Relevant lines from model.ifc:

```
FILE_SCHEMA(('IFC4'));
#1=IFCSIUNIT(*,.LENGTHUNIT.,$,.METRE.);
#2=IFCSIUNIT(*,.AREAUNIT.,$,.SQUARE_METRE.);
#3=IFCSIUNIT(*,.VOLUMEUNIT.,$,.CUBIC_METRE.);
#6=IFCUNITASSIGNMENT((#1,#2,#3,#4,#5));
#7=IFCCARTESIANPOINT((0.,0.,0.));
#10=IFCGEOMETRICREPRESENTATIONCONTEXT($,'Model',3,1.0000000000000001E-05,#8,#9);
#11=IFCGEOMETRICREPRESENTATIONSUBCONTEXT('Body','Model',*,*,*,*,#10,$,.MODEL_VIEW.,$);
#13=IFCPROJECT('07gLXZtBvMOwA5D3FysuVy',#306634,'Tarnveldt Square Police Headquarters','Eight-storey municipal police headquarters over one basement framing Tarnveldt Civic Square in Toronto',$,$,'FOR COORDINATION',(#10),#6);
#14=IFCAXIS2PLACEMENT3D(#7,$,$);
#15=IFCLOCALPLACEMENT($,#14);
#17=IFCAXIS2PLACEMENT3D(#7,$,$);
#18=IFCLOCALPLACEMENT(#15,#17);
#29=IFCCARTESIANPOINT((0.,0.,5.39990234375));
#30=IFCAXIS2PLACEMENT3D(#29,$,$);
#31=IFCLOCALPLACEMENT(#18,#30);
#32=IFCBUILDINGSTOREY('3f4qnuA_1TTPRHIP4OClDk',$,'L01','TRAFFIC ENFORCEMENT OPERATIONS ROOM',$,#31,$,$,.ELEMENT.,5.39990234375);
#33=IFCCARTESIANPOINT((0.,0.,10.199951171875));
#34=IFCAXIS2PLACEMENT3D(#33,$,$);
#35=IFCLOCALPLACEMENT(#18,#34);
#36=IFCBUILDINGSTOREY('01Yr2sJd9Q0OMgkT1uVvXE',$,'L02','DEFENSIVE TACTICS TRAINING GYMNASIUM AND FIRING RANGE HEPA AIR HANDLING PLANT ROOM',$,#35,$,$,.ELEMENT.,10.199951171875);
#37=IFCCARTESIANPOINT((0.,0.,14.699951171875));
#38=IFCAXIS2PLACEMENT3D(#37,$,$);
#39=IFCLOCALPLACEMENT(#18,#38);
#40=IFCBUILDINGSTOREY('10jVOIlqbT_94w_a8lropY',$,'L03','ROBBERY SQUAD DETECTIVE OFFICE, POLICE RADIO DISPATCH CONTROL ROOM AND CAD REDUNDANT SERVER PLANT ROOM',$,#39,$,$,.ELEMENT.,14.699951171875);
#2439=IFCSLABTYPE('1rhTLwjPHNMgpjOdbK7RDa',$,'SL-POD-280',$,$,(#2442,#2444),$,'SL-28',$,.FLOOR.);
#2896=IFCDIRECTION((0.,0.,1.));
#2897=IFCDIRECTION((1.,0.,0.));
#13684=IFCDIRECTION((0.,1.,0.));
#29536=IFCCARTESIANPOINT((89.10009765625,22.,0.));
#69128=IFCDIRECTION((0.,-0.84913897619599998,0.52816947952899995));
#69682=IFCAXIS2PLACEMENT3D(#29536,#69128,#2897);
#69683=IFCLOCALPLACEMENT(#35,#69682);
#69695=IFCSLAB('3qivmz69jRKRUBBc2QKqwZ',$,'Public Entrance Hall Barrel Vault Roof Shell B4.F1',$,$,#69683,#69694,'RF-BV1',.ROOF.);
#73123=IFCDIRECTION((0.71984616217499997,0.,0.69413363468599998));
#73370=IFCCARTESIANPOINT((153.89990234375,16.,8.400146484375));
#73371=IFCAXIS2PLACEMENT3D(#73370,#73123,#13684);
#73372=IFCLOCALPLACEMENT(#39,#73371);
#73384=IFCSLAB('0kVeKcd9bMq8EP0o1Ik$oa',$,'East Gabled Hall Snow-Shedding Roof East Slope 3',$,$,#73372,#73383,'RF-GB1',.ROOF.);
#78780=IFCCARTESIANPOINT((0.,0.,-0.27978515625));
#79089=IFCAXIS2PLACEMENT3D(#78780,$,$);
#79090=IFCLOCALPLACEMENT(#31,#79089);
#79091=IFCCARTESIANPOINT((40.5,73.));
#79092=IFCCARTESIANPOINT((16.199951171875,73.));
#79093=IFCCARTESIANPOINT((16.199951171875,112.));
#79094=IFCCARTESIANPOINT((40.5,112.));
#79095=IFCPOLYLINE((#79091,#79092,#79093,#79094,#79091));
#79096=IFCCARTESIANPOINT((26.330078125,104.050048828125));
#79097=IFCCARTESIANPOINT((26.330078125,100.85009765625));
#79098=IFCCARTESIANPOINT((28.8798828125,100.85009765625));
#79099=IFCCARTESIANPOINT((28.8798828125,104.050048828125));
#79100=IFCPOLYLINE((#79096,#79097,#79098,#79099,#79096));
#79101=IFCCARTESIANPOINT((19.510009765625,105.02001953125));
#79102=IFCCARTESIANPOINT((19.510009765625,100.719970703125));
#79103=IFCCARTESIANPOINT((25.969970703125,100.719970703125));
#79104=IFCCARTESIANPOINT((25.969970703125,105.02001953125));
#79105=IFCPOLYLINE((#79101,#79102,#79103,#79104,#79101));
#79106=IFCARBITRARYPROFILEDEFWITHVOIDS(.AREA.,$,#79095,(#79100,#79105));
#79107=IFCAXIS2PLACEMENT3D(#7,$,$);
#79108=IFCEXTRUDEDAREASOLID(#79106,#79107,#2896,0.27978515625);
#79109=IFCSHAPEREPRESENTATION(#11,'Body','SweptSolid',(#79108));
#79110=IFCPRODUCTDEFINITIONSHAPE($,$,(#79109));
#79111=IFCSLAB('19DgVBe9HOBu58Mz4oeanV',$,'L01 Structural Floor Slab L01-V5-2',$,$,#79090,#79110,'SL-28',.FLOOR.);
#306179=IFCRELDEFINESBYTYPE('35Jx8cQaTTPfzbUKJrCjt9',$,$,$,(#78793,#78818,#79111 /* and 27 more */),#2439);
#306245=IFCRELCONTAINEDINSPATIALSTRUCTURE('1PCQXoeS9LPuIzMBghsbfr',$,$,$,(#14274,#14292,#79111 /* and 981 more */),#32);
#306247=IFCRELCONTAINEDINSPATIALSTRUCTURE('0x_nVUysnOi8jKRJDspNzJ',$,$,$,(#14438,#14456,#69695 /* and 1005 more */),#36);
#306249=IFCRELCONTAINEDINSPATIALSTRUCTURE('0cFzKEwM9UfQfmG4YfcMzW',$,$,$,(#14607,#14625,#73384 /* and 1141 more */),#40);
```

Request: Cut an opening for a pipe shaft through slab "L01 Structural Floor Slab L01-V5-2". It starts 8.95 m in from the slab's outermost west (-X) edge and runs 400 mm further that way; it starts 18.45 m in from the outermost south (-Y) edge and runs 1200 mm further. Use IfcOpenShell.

```python
import numpy as np
import ifcopenshell
import ifcopenshell.api.feature
import ifcopenshell.api.geometry
import ifcopenshell.api.root
import ifcopenshell.geom
import ifcopenshell.util.placement
import ifcopenshell.util.representation
import ifcopenshell.util.shape
import ifcopenshell.util.unit

model = ifcopenshell.open("model.ifc")
unit_scale = ifcopenshell.util.unit.calculate_unit_scale(model)
settings = ifcopenshell.geom.settings()


def volume(element):
    """Net volume in cubic metres, openings subtracted."""
    shape = ifcopenshell.geom.create_shape(settings, element)
    return ifcopenshell.util.shape.get_volume(shape.geometry)


slab = model.by_guid("19DgVBe9HOBu58Mz4oeanV")
before = volume(slab)

# Extent in the slab's own axes, in metres. The edges named are its -X and -Y sides.
slab_shape = ifcopenshell.geom.create_shape(settings, slab)
vertices = ifcopenshell.util.shape.get_vertices(slab_shape.geometry)
x_min, y_min, bottom = vertices.min(axis=0)
top = vertices[:, 2].max()

opening = ifcopenshell.api.root.create_entity(model, ifc_class="IfcOpeningElement", name="Pipe shaft opening", predefined_type="OPENING")
context = ifcopenshell.util.representation.get_context(model, "Model", "Body", "MODEL_VIEW")
width, depth = 0.4, 1.2
outline = [(0.0, 0.0), (width, 0.0), (width, depth), (0.0, depth), (0.0, 0.0)]
# Overshoot both faces by 50 mm so the cut is clean.
shape = ifcopenshell.api.geometry.add_slab_representation(
    model, context=context, depth=top - bottom + 0.1, polyline=outline
)
ifcopenshell.api.geometry.assign_representation(model, product=opening, representation=shape)

matrix = ifcopenshell.util.placement.get_local_placement(slab.ObjectPlacement)
matrix[:, 3] = matrix @ np.append(np.array([x_min + 8.95, y_min + 18.45, bottom - 0.05]) / unit_scale, 1.0)
ifcopenshell.api.geometry.edit_object_placement(model, product=opening, matrix=matrix, is_si=False)
ifcopenshell.api.feature.add_feature(model, feature=opening, element=slab)

after = volume(slab)

print(f"slab volume {before:.3f} -> {after:.3f} m3")

model.write("model_rev.ifc")
```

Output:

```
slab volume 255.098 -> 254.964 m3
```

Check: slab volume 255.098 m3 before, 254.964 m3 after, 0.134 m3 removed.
